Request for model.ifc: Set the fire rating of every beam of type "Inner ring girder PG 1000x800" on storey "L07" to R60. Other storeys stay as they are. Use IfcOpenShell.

First a look at what the model holds.

```python
import ifcopenshell
import ifcopenshell.util.element

model = ifcopenshell.open("model.ifc")
print(model.schema)
storey = next(s for s in model.by_type("IfcBuildingStorey") if s.Name == "L07")
beams = [e for e in ifcopenshell.util.element.get_decomposition(storey) if e.is_a("IfcBeam")]
seen = {}
for e in beams:
    element_type = ifcopenshell.util.element.get_type(e)
    key = (element_type.Name if element_type != e and element_type else None, ifcopenshell.util.element.get_pset(e, "Pset_BeamCommon", "FireRating"))
    seen[key] = seen.get(key, 0) + 1
for (name, value), count in sorted(seen.items(), key=str):
    print(count, "x", name, "|", value)
```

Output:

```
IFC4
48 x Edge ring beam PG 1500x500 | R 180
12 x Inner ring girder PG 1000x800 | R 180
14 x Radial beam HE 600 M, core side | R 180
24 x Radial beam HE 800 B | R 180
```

```python
import ifcopenshell
import ifcopenshell.api.pset
import ifcopenshell.util.element

model = ifcopenshell.open("model.ifc")

storey = next(s for s in model.by_type("IfcBuildingStorey") if s.Name == "L07")
beams = [e for e in ifcopenshell.util.element.get_decomposition(storey) if e.is_a("IfcBeam")]

count = 0
for e in beams:
    element_type = ifcopenshell.util.element.get_type(e)
    if element_type in (None, e) or element_type.Name != "Inner ring girder PG 1000x800":
        continue
    found = ifcopenshell.util.element.get_pset(e, "Pset_BeamCommon", should_inherit=False)
    if found:
        pset = model.by_id(found["id"])
        if len(ifcopenshell.util.element.get_elements_by_pset(pset)) > 1:
            pset = ifcopenshell.api.pset.unshare_pset(model, products=[e], pset=pset)[0]
    else:
        pset = ifcopenshell.api.pset.add_pset(model, product=e, name="Pset_BeamCommon")
    ifcopenshell.api.pset.edit_pset(model, pset=pset, properties={"FireRating": "R60"})
    count += 1

print(count, "beams updated")

model.write("model_updated.ifc")
```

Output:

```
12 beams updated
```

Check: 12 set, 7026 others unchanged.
